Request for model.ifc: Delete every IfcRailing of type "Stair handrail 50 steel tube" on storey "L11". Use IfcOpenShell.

First a look at what the model holds.

```python
import ifcopenshell
import ifcopenshell.util.element

model = ifcopenshell.open("model.ifc")
print(model.schema)
storey = next(s for s in model.by_type("IfcBuildingStorey") if s.Name == "L11")
railings = [e for e in ifcopenshell.util.element.get_decomposition(storey) if e.is_a("IfcRailing")]
seen = {}
for e in railings:
    element_type = ifcopenshell.util.element.get_type(e)
    name = element_type.Name if element_type not in (None, e) else None
    seen[name] = seen.get(name, 0) + 1
for name, count in sorted(seen.items(), key=str):
    print(count, "x", name)
```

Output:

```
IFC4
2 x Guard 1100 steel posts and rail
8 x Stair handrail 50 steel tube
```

```python
import ifcopenshell
import ifcopenshell.api.root
import ifcopenshell.util.element

model = ifcopenshell.open("model.ifc")

storey = next(s for s in model.by_type("IfcBuildingStorey") if s.Name == "L11")
railings = [e for e in ifcopenshell.util.element.get_decomposition(storey) if e.is_a("IfcRailing")]
targets = [e for e in railings if (t := ifcopenshell.util.element.get_type(e)) not in (None, e) and t.Name == "Stair handrail 50 steel tube"]

for e in targets:
    ifcopenshell.api.root.remove_product(model, product=e)
print(len(targets), "removed")

model.write("model_updated.ifc")
```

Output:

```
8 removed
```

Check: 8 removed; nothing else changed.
